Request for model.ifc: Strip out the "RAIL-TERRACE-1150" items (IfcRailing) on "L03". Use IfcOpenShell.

First a look at what the model holds.

```python
import ifcopenshell
import ifcopenshell.util.element

model = ifcopenshell.open("model.ifc")
print(model.schema)
storey = next(s for s in model.by_type("IfcBuildingStorey") if s.Name == "L03")
railings = [e for e in ifcopenshell.util.element.get_decomposition(storey) if e.is_a("IfcRailing")]
seen = {}
for e in railings:
    element_type = ifcopenshell.util.element.get_type(e)
    name = element_type.Name if element_type not in (None, e) else None
    seen[name] = seen.get(name, 0) + 1
for name, count in sorted(seen.items(), key=str):
    print(count, "x", name)
```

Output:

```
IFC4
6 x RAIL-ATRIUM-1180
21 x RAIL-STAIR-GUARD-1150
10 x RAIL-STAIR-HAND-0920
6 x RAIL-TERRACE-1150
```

```python
import ifcopenshell
import ifcopenshell.api.root
import ifcopenshell.util.element

model = ifcopenshell.open("model.ifc")

storey = next(s for s in model.by_type("IfcBuildingStorey") if s.Name == "L03")
railings = [e for e in ifcopenshell.util.element.get_decomposition(storey) if e.is_a("IfcRailing")]
targets = [e for e in railings if (t := ifcopenshell.util.element.get_type(e)) not in (None, e) and t.Name == "RAIL-TERRACE-1150"]

for e in targets:
    ifcopenshell.api.root.remove_product(model, product=e)
print(len(targets), "removed")

model.write("model_updated.ifc")
```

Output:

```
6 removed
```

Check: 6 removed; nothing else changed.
